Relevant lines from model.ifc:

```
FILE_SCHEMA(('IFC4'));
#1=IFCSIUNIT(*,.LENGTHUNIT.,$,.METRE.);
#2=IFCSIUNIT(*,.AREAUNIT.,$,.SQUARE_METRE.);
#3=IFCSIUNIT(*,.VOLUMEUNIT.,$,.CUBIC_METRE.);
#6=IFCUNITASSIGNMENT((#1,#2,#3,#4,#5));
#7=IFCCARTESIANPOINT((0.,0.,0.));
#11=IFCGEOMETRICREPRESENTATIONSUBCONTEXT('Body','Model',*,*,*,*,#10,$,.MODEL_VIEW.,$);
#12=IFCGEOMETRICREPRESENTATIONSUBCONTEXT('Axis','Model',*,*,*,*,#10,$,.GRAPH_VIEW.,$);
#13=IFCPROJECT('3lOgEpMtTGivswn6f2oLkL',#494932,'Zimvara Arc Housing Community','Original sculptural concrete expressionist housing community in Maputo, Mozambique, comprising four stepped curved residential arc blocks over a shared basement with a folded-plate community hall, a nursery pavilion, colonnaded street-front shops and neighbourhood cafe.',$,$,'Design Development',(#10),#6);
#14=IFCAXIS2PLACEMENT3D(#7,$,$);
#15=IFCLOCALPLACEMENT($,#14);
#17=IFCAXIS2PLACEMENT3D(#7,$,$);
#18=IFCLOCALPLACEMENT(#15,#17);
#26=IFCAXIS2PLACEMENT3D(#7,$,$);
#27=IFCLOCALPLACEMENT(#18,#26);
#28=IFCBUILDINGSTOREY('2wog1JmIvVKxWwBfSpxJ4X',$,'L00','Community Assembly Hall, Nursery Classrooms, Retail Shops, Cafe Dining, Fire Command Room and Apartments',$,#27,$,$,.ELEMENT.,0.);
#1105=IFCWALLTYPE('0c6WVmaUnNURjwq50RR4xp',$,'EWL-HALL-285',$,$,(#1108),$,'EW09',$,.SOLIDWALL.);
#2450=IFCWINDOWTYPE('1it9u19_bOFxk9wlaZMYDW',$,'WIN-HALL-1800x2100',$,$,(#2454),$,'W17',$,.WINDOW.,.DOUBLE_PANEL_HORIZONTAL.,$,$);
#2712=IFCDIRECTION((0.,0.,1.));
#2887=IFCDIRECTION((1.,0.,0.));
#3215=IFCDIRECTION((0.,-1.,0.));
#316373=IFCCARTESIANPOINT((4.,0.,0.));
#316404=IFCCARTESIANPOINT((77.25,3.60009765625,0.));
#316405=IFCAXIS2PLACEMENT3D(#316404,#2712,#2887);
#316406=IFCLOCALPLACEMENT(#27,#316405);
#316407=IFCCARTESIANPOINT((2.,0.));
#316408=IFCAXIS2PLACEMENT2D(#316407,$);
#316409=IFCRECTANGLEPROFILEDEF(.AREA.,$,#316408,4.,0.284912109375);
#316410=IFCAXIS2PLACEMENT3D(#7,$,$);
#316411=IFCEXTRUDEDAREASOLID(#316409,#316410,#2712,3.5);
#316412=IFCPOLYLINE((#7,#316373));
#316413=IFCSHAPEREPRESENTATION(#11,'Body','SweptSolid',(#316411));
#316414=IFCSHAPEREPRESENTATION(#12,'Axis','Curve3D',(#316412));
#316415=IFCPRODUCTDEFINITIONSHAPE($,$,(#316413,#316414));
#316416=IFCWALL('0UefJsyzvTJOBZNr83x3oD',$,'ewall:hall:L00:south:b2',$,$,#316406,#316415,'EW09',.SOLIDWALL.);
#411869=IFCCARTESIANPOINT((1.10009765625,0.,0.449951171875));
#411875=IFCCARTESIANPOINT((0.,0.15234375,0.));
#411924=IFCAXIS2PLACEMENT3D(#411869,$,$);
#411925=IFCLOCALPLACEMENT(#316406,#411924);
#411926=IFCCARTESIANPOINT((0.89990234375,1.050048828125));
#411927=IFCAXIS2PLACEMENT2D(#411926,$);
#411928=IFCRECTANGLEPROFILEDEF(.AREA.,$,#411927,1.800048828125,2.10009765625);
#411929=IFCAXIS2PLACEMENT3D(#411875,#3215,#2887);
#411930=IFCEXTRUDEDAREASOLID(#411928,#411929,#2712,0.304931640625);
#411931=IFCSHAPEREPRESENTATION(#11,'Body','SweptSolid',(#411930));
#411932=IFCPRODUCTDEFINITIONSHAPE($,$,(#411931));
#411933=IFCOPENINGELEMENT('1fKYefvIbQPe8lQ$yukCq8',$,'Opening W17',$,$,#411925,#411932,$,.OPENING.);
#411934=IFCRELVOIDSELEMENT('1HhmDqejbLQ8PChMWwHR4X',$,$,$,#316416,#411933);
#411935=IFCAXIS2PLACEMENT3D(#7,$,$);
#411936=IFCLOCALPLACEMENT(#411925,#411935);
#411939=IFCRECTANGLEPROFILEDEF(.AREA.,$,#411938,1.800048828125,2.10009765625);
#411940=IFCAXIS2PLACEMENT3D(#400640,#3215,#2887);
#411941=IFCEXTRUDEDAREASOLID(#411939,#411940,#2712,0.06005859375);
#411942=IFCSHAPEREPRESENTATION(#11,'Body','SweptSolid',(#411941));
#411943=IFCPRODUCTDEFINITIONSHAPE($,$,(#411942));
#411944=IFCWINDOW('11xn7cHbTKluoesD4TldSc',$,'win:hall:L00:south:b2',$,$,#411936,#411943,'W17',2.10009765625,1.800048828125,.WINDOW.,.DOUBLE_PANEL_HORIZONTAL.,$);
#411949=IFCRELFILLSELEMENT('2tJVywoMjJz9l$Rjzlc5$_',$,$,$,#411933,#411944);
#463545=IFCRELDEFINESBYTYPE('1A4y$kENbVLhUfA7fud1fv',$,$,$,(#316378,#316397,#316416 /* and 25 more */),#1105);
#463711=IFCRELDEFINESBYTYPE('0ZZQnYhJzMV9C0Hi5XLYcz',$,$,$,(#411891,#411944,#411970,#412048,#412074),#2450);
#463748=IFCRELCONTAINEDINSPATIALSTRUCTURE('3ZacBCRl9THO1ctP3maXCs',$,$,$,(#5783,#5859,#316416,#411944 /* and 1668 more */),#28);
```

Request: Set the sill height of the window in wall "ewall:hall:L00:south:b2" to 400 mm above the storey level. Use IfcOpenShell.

```python
import numpy as np
import ifcopenshell
import ifcopenshell.api.geometry
import ifcopenshell.geom
import ifcopenshell.util.element
import ifcopenshell.util.placement
import ifcopenshell.util.shape
import ifcopenshell.util.unit

model = ifcopenshell.open("model.ifc")
unit_scale = ifcopenshell.util.unit.calculate_unit_scale(model)

window = model.by_id(411944)
opening = window.FillsVoids[0].RelatingOpeningElement
storey = ifcopenshell.util.element.get_container(window, ifc_class="IfcBuildingStorey")
level = ifcopenshell.util.placement.get_local_placement(storey.ObjectPlacement)[2, 3]

# The opening's origin need not be at the sill, so measure its lowest point.
shape = ifcopenshell.geom.create_shape(ifcopenshell.geom.settings(), opening)
bottom = ifcopenshell.util.shape.get_shape_bottom_elevation(shape, shape.geometry) / unit_scale
dz = level + 0.4 - bottom

shift = np.array([0.0, 0.0, dz])
# The window is placed relative to its opening, so it follows when the opening moves.
matrix = ifcopenshell.util.placement.get_local_placement(opening.ObjectPlacement)
matrix[:3, 3] += shift
ifcopenshell.api.geometry.edit_object_placement(
    model, product=opening, matrix=matrix, is_si=False, should_transform_children=True
)

print(f"moved by {dz * unit_scale:+.3f} m")

model.write("model_edited.ifc")
```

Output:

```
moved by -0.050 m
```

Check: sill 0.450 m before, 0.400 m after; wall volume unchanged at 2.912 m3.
